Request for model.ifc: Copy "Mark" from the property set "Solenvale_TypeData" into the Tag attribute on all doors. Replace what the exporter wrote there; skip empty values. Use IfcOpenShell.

First a look at what the model holds.

```python
import ifcopenshell
import ifcopenshell.util.element

model = ifcopenshell.open("model.ifc")
print(model.schema)
doors = model.by_type("IfcDoor")
print(len(doors), "doors")
for e in doors[:8]:
    source = ifcopenshell.util.element.get_pset(e, "Solenvale_TypeData", "Mark")
    target = e.Tag
    print(e.id(), repr(source), repr(target), sep=" | ")
```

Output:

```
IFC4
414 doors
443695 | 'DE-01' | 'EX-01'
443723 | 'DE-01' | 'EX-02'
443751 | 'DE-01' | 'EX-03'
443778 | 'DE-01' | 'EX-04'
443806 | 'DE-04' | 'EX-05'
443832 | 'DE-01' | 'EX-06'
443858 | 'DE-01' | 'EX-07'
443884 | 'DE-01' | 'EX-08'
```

```python
import ifcopenshell
import ifcopenshell.util.element

model = ifcopenshell.open("model.ifc")

count = 0
for e in model.by_type("IfcDoor"):
    value = ifcopenshell.util.element.get_pset(e, "Solenvale_TypeData", "Mark")
    current = e.Tag
    if not value or not value.strip() or current == value:
        continue
    e.Tag = value
    count += 1

print(count, "doors updated")

model.write("model_updated.ifc")
```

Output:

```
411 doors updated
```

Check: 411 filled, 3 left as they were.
